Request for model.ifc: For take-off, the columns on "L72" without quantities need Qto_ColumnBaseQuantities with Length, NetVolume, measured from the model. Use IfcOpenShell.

First a look at what the model holds.

```python
import ifcopenshell
import ifcopenshell.util.element
import ifcopenshell.util.unit

model = ifcopenshell.open("model.ifc")
print(model.schema)
for unit_type in ("LENGTHUNIT", "AREAUNIT", "VOLUMEUNIT"):
    print(unit_type, ifcopenshell.util.unit.calculate_unit_scale(model, unit_type))
storey = next(s for s in model.by_type("IfcBuildingStorey") if s.Name == "L72")
columns = [e for e in ifcopenshell.util.element.get_decomposition(storey) if e.is_a("IfcColumn")]
for e in sorted(columns, key=lambda e: e.id()):
    print(e.id(), e.is_a(), e.Name, list(ifcopenshell.util.element.get_psets(e, qtos_only=True)), sep=" | ")
```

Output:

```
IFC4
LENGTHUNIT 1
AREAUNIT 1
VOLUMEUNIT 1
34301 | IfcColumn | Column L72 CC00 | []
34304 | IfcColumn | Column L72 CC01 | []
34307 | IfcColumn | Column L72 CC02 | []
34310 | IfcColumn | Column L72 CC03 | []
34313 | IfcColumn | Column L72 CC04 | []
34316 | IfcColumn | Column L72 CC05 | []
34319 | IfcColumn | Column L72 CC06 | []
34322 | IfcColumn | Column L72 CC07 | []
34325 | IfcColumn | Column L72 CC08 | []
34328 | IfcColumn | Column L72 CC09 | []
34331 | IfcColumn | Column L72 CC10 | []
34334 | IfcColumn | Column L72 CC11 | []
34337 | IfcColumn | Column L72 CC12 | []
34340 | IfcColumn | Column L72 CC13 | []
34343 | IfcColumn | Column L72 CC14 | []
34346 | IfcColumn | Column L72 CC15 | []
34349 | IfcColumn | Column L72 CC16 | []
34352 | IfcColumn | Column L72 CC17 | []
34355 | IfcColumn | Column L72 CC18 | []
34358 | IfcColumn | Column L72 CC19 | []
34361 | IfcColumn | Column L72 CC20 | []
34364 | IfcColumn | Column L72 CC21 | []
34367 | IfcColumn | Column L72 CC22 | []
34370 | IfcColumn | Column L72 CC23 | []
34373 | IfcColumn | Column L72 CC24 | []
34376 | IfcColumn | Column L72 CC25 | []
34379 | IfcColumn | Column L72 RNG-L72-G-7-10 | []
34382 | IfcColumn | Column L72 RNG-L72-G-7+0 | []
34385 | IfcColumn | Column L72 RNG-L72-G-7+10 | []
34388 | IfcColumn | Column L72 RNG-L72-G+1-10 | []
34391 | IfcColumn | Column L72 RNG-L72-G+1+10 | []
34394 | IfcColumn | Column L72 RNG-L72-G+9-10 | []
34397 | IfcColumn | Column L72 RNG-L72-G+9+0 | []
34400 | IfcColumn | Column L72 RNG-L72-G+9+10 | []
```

```python
import ifcopenshell
import ifcopenshell.api.pset
import ifcopenshell.geom
import ifcopenshell.util.element
import ifcopenshell.util.shape
import ifcopenshell.util.unit

model = ifcopenshell.open("model.ifc")
unit_scale = ifcopenshell.util.unit.calculate_unit_scale(model)
volume_scale = ifcopenshell.util.unit.calculate_unit_scale(model, "VOLUMEUNIT")
settings = ifcopenshell.geom.settings()

storey = next(s for s in model.by_type("IfcBuildingStorey") if s.Name == "L72")
columns = [e for e in ifcopenshell.util.element.get_decomposition(storey) if e.is_a("IfcColumn")]

for e in sorted(columns, key=lambda e: e.id()):
    if ifcopenshell.util.element.get_psets(e, qtos_only=True, should_inherit=False):
        continue
    # Geometry comes back in metres, in the element's own axes.
    shape = ifcopenshell.geom.create_shape(settings, e)
    values = {
        "Length": ifcopenshell.util.shape.get_z(shape.geometry) / unit_scale,
        "NetVolume": ifcopenshell.util.shape.get_volume(shape.geometry) / volume_scale,
    }
    qto = ifcopenshell.api.pset.add_qto(model, product=e, name="Qto_ColumnBaseQuantities")
    ifcopenshell.api.pset.edit_qto(model, qto=qto, properties=values)
    print(e.id(), {k: round(v, 3) for k, v in values.items()})

model.write("model_edited.ifc")
```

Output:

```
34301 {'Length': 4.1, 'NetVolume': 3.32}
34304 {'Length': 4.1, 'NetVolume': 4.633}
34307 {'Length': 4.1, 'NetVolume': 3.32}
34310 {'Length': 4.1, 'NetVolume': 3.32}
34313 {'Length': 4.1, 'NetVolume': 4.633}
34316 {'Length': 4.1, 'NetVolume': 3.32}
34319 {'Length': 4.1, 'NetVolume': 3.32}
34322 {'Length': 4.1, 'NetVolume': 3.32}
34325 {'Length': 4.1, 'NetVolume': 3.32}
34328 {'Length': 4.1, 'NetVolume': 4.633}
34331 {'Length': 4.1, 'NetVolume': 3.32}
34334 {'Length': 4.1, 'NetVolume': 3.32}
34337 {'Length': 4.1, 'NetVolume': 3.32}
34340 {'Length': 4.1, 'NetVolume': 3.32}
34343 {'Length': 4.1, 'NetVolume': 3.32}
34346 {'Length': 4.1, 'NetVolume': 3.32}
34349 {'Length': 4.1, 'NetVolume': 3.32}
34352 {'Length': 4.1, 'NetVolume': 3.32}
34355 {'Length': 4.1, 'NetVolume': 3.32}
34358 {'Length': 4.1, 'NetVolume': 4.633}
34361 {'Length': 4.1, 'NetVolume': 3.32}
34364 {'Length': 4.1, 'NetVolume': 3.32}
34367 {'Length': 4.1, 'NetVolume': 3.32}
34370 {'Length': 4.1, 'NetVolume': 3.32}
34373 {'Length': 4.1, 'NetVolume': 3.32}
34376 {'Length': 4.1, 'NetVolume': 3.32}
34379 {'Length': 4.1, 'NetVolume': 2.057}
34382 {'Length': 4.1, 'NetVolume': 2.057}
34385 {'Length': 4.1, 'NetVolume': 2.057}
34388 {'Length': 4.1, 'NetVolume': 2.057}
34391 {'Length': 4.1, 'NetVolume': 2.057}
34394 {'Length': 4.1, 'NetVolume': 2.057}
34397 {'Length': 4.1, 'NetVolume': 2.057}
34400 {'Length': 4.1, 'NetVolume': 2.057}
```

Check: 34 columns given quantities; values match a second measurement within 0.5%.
